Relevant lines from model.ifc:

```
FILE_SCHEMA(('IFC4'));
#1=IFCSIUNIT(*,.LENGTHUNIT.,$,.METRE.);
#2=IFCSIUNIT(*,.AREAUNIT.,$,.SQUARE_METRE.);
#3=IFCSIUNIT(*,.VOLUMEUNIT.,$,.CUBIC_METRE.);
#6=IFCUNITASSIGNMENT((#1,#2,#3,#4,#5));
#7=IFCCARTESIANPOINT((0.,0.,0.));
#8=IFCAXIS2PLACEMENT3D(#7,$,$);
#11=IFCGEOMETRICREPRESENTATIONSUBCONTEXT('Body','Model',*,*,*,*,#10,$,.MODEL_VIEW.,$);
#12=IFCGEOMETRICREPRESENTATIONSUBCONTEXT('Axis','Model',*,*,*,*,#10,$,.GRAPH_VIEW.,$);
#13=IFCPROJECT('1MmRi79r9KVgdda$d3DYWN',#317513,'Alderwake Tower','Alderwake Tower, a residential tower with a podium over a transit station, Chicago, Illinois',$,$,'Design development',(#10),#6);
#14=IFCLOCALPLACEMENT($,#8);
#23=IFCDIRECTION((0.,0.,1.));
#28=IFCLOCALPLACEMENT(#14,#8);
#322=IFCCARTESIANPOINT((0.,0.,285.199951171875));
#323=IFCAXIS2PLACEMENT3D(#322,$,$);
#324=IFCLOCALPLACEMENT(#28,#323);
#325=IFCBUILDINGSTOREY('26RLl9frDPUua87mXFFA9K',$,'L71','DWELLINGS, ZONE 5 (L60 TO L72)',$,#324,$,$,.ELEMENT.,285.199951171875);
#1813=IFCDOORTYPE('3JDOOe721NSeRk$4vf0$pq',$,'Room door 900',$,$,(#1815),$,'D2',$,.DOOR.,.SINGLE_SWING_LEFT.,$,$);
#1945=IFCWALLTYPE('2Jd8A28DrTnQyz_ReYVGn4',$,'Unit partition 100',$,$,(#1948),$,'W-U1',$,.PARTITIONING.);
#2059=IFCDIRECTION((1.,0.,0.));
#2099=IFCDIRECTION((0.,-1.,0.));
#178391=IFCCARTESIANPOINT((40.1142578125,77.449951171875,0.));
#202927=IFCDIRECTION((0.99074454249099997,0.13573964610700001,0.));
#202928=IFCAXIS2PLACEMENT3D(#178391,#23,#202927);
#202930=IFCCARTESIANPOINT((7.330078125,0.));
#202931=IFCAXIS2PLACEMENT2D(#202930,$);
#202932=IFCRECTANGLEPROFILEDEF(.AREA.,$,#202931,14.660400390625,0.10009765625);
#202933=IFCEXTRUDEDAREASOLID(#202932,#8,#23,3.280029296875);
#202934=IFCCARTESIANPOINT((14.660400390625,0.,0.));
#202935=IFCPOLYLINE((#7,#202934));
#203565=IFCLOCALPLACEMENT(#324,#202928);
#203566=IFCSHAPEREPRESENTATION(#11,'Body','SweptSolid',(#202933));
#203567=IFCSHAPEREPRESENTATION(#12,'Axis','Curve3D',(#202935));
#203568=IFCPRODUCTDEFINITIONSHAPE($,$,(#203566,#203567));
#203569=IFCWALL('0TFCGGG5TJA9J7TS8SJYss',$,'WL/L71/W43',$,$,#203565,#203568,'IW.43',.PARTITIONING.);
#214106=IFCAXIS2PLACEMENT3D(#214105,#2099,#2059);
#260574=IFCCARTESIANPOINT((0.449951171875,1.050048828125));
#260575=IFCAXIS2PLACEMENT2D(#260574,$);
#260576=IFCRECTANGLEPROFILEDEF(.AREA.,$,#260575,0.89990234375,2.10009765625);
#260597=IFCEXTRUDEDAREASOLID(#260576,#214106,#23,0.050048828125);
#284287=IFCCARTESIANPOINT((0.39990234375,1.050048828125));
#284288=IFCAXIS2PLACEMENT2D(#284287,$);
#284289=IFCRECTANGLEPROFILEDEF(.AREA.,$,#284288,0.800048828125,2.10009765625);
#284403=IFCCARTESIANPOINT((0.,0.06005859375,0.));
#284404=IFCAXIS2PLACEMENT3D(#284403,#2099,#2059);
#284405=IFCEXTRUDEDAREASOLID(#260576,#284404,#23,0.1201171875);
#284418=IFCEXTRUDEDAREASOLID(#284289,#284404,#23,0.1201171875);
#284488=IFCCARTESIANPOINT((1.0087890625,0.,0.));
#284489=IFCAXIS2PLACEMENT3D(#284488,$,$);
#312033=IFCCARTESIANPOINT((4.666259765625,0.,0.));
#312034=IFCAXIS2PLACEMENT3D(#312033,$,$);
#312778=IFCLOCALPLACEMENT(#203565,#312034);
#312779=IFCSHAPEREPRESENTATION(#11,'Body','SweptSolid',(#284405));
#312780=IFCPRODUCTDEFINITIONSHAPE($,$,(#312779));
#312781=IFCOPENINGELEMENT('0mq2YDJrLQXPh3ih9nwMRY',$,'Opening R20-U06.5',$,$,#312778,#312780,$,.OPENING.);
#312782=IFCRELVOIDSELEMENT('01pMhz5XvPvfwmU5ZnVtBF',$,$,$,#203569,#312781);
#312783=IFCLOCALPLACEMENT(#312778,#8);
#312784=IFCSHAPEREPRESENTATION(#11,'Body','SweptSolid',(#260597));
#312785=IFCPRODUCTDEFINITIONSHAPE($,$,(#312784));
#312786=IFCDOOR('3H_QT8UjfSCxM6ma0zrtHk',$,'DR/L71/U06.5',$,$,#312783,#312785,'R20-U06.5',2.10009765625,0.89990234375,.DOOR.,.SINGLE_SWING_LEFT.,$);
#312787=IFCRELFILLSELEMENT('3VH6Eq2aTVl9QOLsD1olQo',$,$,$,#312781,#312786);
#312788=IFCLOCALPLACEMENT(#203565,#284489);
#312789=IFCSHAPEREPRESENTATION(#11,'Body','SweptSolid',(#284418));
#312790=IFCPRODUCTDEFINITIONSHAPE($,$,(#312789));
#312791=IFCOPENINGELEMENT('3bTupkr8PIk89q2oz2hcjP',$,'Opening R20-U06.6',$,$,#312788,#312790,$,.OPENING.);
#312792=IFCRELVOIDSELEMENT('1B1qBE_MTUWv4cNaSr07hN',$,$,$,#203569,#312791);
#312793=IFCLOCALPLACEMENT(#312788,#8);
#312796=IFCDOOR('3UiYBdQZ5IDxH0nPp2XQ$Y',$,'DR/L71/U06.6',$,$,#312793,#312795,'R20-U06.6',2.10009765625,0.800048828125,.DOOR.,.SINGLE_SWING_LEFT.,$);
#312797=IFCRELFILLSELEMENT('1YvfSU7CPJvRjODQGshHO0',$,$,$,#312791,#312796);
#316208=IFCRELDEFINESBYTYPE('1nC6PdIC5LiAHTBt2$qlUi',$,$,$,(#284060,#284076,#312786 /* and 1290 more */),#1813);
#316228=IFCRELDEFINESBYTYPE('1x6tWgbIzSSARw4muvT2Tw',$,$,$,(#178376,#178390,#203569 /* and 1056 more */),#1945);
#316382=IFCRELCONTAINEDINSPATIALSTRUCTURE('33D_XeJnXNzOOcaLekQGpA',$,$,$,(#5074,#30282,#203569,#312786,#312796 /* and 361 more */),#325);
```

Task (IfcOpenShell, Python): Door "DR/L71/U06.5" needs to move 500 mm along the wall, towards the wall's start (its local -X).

```python
import ifcopenshell
import ifcopenshell.api.geometry
import ifcopenshell.util.placement

model = ifcopenshell.open("model.ifc")

door = model.by_guid("3H_QT8UjfSCxM6ma0zrtHk")
opening = door.FillsVoids[0].RelatingOpeningElement
wall = opening.VoidsElements[0].RelatingBuildingElement

wall_matrix = ifcopenshell.util.placement.get_local_placement(wall.ObjectPlacement)
shift = wall_matrix[:3, 0] * -0.5
before = ifcopenshell.util.placement.get_local_placement(door.ObjectPlacement)[:3, 3].copy()

# The door is placed relative to its opening, so it follows when the opening moves.
matrix = ifcopenshell.util.placement.get_local_placement(opening.ObjectPlacement)
matrix[:3, 3] += shift
ifcopenshell.api.geometry.edit_object_placement(
    model, product=opening, matrix=matrix, is_si=False, should_transform_children=True
)

after = ifcopenshell.util.placement.get_local_placement(door.ObjectPlacement)[:3, 3]
print("door moved by", (after - before).round(3) + 0.0)

model.write("model_v2.ifc")
```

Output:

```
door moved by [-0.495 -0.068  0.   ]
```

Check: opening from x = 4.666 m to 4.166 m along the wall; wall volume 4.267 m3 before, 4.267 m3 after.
